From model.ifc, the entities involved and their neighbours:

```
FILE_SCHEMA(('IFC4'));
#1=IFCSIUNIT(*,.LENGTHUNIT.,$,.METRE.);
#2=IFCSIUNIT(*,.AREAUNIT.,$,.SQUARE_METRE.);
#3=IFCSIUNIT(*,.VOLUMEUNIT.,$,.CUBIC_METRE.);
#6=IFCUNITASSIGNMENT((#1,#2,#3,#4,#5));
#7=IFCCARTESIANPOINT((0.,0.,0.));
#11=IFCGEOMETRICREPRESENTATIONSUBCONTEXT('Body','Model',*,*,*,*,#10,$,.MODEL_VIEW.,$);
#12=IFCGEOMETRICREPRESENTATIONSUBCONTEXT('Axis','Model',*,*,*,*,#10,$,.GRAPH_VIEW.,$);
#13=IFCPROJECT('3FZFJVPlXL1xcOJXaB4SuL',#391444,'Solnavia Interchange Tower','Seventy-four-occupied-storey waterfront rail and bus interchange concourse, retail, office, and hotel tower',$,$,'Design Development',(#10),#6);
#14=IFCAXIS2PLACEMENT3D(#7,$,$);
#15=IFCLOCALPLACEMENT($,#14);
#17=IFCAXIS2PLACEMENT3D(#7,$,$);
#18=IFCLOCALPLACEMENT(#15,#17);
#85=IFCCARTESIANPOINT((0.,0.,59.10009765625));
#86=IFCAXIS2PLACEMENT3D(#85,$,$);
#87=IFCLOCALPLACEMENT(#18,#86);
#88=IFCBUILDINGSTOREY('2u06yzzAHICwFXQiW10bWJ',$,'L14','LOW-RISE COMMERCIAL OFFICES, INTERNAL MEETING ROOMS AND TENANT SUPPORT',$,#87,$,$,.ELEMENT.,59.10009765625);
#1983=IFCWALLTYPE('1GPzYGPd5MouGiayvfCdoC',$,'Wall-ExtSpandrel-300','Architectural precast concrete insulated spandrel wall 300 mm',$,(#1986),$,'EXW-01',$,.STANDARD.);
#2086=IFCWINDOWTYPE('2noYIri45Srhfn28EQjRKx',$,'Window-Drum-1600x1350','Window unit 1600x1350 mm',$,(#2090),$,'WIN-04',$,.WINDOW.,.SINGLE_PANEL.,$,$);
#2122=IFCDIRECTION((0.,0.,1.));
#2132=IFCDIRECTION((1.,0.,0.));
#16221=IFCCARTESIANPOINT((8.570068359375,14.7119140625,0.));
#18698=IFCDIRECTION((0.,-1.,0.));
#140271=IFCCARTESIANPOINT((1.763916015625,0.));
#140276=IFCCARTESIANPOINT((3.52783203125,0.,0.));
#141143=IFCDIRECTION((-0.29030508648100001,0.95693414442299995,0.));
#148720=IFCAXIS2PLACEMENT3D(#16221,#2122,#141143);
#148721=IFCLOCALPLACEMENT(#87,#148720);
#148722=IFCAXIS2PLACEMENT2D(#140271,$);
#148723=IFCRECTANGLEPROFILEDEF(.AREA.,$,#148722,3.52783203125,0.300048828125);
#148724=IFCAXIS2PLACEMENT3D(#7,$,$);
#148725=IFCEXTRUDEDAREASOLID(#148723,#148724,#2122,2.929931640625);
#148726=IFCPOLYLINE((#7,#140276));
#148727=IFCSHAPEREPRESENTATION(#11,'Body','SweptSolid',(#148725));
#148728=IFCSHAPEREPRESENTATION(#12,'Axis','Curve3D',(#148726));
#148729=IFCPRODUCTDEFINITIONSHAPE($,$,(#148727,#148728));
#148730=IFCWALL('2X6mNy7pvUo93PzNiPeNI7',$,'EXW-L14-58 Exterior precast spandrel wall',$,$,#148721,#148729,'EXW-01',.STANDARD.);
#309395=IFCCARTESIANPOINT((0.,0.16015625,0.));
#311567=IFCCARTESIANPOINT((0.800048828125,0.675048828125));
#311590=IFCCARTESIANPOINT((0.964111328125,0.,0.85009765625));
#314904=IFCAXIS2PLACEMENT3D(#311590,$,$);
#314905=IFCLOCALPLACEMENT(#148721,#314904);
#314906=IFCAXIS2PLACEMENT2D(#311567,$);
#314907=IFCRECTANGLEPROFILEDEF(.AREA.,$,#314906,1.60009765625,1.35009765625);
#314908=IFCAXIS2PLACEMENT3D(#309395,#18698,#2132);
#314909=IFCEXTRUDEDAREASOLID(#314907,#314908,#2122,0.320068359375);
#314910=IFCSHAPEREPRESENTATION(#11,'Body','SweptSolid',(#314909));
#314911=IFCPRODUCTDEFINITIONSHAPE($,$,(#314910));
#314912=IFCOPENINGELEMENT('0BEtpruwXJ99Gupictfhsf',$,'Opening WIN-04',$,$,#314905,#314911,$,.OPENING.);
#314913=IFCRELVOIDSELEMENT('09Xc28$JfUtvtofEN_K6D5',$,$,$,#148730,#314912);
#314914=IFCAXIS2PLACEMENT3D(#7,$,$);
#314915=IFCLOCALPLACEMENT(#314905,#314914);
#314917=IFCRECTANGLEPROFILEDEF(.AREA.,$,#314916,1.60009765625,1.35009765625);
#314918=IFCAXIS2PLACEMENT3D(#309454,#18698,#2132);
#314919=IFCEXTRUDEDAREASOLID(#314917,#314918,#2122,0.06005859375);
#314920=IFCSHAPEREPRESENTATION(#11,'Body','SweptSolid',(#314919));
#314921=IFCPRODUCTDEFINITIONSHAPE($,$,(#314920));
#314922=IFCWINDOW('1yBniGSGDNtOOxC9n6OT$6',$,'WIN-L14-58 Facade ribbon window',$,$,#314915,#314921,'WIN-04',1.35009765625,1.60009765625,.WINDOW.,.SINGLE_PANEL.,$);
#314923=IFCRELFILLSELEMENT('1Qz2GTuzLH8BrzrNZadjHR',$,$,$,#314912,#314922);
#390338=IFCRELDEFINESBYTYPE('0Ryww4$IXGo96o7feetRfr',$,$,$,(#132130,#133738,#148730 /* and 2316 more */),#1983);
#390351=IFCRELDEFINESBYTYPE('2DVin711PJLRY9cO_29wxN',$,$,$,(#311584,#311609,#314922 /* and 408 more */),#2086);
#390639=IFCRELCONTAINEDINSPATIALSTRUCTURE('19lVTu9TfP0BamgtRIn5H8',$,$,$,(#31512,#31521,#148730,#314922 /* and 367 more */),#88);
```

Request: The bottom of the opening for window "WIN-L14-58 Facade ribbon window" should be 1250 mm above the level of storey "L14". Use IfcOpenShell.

```python
import numpy as np
import ifcopenshell
import ifcopenshell.api.geometry
import ifcopenshell.geom
import ifcopenshell.util.element
import ifcopenshell.util.placement
import ifcopenshell.util.shape
import ifcopenshell.util.unit

model = ifcopenshell.open("model.ifc")
unit_scale = ifcopenshell.util.unit.calculate_unit_scale(model)

window = model.by_guid("1yBniGSGDNtOOxC9n6OT$6")
opening = window.FillsVoids[0].RelatingOpeningElement
storey = ifcopenshell.util.element.get_container(window, ifc_class="IfcBuildingStorey")
level = ifcopenshell.util.placement.get_local_placement(storey.ObjectPlacement)[2, 3]

# The opening's origin need not be at the sill, so measure its lowest point.
shape = ifcopenshell.geom.create_shape(ifcopenshell.geom.settings(), opening)
bottom = ifcopenshell.util.shape.get_shape_bottom_elevation(shape, shape.geometry) / unit_scale
dz = level + 1.25 / unit_scale - bottom

shift = np.array([0.0, 0.0, dz])
# The window is placed relative to its opening, so it follows when the opening moves.
matrix = ifcopenshell.util.placement.get_local_placement(opening.ObjectPlacement)
matrix[:3, 3] += shift
ifcopenshell.api.geometry.edit_object_placement(
    model, product=opening, matrix=matrix, is_si=False, should_transform_children=True
)

print(f"moved by {dz * unit_scale:+.3f} m")

model.write("model_updated.ifc")
```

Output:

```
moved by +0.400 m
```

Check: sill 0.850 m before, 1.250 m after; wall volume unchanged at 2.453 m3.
